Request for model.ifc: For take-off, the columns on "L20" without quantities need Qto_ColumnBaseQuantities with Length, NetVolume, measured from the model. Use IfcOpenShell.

First a look at what the model holds.

```python
import ifcopenshell
import ifcopenshell.util.element
import ifcopenshell.util.unit

model = ifcopenshell.open("model.ifc")
print(model.schema)
for unit_type in ("LENGTHUNIT", "AREAUNIT", "VOLUMEUNIT"):
    print(unit_type, ifcopenshell.util.unit.calculate_unit_scale(model, unit_type))
storey = next(s for s in model.by_type("IfcBuildingStorey") if s.Name == "L20")
columns = [e for e in ifcopenshell.util.element.get_decomposition(storey) if e.is_a("IfcColumn")]
for e in sorted(columns, key=lambda e: e.id()):
    print(e.id(), e.is_a(), e.Name, list(ifcopenshell.util.element.get_psets(e, qtos_only=True)), sep=" | ")
```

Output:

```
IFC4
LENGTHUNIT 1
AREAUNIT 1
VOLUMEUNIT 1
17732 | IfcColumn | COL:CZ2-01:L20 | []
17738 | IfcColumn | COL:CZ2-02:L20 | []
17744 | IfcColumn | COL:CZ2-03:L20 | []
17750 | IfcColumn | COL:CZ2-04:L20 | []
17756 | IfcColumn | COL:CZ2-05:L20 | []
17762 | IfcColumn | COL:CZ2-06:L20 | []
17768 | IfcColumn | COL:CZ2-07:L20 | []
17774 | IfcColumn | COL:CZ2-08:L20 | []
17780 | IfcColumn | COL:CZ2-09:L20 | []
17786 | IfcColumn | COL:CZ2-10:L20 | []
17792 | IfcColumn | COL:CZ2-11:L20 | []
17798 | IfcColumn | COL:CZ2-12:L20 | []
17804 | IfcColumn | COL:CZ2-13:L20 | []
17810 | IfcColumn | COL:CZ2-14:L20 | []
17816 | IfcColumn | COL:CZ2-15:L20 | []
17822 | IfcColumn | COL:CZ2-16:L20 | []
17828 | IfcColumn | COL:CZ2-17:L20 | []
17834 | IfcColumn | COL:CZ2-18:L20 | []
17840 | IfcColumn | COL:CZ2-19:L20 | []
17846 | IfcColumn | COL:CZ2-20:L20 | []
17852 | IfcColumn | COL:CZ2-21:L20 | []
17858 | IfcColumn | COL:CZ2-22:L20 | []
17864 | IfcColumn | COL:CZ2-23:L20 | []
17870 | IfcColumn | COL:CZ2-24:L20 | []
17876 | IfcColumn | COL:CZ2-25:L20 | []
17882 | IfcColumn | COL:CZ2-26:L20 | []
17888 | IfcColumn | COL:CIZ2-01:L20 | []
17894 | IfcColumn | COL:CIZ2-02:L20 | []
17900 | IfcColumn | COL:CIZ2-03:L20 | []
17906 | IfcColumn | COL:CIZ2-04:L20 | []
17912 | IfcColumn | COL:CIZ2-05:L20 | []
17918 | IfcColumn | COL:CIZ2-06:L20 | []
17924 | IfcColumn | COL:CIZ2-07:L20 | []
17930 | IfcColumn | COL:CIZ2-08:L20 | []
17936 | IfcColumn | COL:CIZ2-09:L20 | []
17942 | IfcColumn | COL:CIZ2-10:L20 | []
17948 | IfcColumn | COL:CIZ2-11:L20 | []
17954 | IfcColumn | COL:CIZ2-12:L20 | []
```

```python
import ifcopenshell
import ifcopenshell.api.pset
import ifcopenshell.geom
import ifcopenshell.util.element
import ifcopenshell.util.shape
import ifcopenshell.util.unit

model = ifcopenshell.open("model.ifc")
unit_scale = ifcopenshell.util.unit.calculate_unit_scale(model)
volume_scale = ifcopenshell.util.unit.calculate_unit_scale(model, "VOLUMEUNIT")
settings = ifcopenshell.geom.settings()

storey = next(s for s in model.by_type("IfcBuildingStorey") if s.Name == "L20")
columns = [e for e in ifcopenshell.util.element.get_decomposition(storey) if e.is_a("IfcColumn")]

for e in sorted(columns, key=lambda e: e.id()):
    if ifcopenshell.util.element.get_psets(e, qtos_only=True, should_inherit=False):
        continue
    # Geometry comes back in metres, in the element's own axes.
    shape = ifcopenshell.geom.create_shape(settings, e)
    values = {
        "Length": ifcopenshell.util.shape.get_z(shape.geometry) / unit_scale,
        "NetVolume": ifcopenshell.util.shape.get_volume(shape.geometry) / volume_scale,
    }
    qto = ifcopenshell.api.pset.add_qto(model, product=e, name="Qto_ColumnBaseQuantities")
    ifcopenshell.api.pset.edit_qto(model, qto=qto, properties=values)
    print(e.id(), {k: round(v, 3) for k, v in values.items()})

model.write("model_rev.ifc")
```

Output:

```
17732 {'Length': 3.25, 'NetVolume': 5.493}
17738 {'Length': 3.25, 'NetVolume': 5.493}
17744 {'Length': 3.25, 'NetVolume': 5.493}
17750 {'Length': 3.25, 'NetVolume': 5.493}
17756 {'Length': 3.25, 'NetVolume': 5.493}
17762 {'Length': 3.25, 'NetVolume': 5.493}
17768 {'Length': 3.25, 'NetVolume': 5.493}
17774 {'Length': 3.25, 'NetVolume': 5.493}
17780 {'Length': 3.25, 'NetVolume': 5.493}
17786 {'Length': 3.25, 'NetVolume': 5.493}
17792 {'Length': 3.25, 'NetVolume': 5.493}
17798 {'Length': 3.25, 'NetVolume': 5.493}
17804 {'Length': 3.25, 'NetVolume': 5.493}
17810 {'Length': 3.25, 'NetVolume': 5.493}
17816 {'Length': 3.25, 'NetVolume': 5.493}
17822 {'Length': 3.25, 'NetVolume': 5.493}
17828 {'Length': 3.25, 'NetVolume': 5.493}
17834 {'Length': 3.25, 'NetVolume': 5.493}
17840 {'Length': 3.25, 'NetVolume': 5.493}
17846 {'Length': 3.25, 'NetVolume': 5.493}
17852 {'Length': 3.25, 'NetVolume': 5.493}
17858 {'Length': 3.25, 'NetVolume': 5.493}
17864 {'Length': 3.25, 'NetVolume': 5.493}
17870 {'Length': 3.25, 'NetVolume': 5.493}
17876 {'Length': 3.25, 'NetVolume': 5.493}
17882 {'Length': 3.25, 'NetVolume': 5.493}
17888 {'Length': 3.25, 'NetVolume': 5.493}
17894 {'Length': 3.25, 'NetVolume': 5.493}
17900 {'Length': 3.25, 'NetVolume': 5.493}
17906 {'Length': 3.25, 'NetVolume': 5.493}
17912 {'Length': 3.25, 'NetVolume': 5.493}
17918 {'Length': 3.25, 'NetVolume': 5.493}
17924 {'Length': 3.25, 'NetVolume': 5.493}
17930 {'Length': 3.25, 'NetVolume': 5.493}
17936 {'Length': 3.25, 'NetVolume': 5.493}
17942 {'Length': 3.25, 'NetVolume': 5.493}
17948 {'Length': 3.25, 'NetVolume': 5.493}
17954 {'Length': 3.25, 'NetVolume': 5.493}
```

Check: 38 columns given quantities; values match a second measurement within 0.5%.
